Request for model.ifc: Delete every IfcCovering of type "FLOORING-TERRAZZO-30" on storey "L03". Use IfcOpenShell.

First a look at what the model holds.

```python
import ifcopenshell
import ifcopenshell.util.element

model = ifcopenshell.open("model.ifc")
print(model.schema)
storey = next(s for s in model.by_type("IfcBuildingStorey") if s.Name == "L03")
coverings = [e for e in ifcopenshell.util.element.get_decomposition(storey) if e.is_a("IfcCovering")]
seen = {}
for e in coverings:
    element_type = ifcopenshell.util.element.get_type(e)
    name = element_type.Name if element_type not in (None, e) else None
    seen[name] = seen.get(name, 0) + 1
for name, count in sorted(seen.items(), key=str):
    print(count, "x", name)
```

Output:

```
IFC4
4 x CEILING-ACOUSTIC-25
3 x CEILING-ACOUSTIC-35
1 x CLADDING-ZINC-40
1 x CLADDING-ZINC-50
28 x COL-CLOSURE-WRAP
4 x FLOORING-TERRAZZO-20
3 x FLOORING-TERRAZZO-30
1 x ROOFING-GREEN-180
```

```python
import ifcopenshell
import ifcopenshell.api.root
import ifcopenshell.util.element

model = ifcopenshell.open("model.ifc")

storey = next(s for s in model.by_type("IfcBuildingStorey") if s.Name == "L03")
coverings = [e for e in ifcopenshell.util.element.get_decomposition(storey) if e.is_a("IfcCovering")]
targets = [e for e in coverings if (t := ifcopenshell.util.element.get_type(e)) not in (None, e) and t.Name == "FLOORING-TERRAZZO-30"]

for e in targets:
    ifcopenshell.api.root.remove_product(model, product=e)
print(len(targets), "removed")

model.write("model_updated.ifc")
```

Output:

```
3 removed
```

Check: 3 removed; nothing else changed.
